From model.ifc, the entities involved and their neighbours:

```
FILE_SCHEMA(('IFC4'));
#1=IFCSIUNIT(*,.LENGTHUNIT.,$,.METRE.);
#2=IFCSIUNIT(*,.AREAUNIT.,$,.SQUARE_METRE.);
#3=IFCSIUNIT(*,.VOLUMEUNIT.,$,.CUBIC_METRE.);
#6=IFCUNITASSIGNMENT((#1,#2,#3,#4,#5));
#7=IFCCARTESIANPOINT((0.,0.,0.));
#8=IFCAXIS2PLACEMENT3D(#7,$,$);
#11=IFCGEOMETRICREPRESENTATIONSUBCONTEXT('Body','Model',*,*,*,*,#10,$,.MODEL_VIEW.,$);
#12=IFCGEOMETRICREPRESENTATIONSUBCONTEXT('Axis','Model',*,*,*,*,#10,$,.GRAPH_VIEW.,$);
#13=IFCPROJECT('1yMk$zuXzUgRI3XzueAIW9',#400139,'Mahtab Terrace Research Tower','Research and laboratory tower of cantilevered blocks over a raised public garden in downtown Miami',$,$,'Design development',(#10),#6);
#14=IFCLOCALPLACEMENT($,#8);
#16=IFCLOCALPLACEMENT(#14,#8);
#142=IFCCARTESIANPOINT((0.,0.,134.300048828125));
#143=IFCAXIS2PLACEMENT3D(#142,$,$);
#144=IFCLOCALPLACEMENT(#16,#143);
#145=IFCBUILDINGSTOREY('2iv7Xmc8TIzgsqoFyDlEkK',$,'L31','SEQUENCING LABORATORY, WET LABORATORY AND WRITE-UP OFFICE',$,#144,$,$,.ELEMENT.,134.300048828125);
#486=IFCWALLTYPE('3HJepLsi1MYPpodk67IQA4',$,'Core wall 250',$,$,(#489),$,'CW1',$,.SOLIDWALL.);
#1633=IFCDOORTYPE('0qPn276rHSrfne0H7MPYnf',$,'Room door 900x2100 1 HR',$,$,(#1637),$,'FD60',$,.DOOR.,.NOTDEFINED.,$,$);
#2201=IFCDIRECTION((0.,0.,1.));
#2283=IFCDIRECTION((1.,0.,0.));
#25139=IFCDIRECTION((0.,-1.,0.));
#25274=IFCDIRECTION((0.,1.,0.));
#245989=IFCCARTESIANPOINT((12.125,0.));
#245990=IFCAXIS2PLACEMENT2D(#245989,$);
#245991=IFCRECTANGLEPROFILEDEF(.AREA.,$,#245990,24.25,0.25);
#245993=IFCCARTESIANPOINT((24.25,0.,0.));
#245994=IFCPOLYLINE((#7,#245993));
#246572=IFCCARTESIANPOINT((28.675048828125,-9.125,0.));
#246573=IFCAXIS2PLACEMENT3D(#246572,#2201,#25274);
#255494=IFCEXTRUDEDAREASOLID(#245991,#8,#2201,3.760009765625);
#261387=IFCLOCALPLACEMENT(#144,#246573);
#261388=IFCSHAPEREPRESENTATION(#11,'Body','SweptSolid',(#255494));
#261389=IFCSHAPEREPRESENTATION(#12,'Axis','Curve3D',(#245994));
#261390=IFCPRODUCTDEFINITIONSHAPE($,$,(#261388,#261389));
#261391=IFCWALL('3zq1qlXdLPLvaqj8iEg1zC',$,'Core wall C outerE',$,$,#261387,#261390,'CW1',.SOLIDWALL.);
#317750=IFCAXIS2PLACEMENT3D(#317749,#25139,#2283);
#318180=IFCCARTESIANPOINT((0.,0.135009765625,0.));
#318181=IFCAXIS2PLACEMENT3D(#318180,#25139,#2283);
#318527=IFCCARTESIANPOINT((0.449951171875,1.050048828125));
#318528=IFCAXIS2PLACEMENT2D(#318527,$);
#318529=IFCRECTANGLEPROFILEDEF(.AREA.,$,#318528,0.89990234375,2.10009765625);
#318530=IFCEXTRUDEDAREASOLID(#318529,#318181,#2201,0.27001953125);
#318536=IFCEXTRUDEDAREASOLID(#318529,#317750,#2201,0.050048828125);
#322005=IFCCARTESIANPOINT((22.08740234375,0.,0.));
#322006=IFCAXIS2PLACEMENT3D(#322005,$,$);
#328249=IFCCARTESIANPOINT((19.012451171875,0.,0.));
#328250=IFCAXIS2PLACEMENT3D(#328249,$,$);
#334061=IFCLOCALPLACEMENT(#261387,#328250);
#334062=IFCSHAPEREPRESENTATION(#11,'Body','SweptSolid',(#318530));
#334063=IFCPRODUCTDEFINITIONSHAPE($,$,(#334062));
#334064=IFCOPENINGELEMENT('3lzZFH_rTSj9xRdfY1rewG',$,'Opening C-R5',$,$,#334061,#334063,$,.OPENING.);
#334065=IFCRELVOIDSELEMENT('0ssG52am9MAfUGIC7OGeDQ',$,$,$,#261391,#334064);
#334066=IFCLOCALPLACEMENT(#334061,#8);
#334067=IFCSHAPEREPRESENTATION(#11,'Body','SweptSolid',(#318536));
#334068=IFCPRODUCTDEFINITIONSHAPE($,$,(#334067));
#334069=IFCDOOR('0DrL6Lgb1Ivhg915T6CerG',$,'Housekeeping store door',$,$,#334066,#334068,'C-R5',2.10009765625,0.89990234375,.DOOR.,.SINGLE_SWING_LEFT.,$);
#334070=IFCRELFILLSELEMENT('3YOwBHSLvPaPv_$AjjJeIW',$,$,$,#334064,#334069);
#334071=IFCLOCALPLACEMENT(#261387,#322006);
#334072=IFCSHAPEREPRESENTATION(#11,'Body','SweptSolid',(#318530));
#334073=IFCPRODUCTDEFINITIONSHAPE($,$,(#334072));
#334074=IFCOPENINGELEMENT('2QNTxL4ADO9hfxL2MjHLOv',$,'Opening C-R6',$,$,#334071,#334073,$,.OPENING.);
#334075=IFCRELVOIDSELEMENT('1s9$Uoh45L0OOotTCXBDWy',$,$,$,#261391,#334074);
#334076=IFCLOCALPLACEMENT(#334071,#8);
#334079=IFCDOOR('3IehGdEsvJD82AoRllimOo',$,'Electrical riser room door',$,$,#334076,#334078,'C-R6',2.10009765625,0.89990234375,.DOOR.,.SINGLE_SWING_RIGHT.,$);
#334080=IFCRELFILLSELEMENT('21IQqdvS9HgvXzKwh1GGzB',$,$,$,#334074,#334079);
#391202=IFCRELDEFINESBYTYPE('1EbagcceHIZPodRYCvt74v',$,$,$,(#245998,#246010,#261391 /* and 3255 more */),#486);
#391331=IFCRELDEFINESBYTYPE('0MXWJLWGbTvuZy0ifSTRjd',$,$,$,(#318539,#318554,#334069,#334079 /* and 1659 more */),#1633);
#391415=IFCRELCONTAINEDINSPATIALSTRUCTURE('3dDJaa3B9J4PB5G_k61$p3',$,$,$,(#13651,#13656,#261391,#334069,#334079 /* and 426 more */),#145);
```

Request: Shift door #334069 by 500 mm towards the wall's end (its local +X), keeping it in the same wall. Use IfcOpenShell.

```python
import ifcopenshell
import ifcopenshell.api.geometry
import ifcopenshell.util.placement
import ifcopenshell.util.unit

model = ifcopenshell.open("model.ifc")
unit_scale = ifcopenshell.util.unit.calculate_unit_scale(model)

door = model.by_guid("0DrL6Lgb1Ivhg915T6CerG")
opening = door.FillsVoids[0].RelatingOpeningElement
wall = opening.VoidsElements[0].RelatingBuildingElement

wall_matrix = ifcopenshell.util.placement.get_local_placement(wall.ObjectPlacement)
shift = wall_matrix[:3, 0] * 0.5 / unit_scale
before = ifcopenshell.util.placement.get_local_placement(door.ObjectPlacement)[:3, 3].copy()

# The door is placed relative to its opening, so it follows when the opening moves.
matrix = ifcopenshell.util.placement.get_local_placement(opening.ObjectPlacement)
matrix[:3, 3] += shift
ifcopenshell.api.geometry.edit_object_placement(
    model, product=opening, matrix=matrix, is_si=False, should_transform_children=True
)

after = ifcopenshell.util.placement.get_local_placement(door.ObjectPlacement)[:3, 3]
print("door moved by", (after - before).round(3) + 0.0)

model.write("model_v2.ifc")
```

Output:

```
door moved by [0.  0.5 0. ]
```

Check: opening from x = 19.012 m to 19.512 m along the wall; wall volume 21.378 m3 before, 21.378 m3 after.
